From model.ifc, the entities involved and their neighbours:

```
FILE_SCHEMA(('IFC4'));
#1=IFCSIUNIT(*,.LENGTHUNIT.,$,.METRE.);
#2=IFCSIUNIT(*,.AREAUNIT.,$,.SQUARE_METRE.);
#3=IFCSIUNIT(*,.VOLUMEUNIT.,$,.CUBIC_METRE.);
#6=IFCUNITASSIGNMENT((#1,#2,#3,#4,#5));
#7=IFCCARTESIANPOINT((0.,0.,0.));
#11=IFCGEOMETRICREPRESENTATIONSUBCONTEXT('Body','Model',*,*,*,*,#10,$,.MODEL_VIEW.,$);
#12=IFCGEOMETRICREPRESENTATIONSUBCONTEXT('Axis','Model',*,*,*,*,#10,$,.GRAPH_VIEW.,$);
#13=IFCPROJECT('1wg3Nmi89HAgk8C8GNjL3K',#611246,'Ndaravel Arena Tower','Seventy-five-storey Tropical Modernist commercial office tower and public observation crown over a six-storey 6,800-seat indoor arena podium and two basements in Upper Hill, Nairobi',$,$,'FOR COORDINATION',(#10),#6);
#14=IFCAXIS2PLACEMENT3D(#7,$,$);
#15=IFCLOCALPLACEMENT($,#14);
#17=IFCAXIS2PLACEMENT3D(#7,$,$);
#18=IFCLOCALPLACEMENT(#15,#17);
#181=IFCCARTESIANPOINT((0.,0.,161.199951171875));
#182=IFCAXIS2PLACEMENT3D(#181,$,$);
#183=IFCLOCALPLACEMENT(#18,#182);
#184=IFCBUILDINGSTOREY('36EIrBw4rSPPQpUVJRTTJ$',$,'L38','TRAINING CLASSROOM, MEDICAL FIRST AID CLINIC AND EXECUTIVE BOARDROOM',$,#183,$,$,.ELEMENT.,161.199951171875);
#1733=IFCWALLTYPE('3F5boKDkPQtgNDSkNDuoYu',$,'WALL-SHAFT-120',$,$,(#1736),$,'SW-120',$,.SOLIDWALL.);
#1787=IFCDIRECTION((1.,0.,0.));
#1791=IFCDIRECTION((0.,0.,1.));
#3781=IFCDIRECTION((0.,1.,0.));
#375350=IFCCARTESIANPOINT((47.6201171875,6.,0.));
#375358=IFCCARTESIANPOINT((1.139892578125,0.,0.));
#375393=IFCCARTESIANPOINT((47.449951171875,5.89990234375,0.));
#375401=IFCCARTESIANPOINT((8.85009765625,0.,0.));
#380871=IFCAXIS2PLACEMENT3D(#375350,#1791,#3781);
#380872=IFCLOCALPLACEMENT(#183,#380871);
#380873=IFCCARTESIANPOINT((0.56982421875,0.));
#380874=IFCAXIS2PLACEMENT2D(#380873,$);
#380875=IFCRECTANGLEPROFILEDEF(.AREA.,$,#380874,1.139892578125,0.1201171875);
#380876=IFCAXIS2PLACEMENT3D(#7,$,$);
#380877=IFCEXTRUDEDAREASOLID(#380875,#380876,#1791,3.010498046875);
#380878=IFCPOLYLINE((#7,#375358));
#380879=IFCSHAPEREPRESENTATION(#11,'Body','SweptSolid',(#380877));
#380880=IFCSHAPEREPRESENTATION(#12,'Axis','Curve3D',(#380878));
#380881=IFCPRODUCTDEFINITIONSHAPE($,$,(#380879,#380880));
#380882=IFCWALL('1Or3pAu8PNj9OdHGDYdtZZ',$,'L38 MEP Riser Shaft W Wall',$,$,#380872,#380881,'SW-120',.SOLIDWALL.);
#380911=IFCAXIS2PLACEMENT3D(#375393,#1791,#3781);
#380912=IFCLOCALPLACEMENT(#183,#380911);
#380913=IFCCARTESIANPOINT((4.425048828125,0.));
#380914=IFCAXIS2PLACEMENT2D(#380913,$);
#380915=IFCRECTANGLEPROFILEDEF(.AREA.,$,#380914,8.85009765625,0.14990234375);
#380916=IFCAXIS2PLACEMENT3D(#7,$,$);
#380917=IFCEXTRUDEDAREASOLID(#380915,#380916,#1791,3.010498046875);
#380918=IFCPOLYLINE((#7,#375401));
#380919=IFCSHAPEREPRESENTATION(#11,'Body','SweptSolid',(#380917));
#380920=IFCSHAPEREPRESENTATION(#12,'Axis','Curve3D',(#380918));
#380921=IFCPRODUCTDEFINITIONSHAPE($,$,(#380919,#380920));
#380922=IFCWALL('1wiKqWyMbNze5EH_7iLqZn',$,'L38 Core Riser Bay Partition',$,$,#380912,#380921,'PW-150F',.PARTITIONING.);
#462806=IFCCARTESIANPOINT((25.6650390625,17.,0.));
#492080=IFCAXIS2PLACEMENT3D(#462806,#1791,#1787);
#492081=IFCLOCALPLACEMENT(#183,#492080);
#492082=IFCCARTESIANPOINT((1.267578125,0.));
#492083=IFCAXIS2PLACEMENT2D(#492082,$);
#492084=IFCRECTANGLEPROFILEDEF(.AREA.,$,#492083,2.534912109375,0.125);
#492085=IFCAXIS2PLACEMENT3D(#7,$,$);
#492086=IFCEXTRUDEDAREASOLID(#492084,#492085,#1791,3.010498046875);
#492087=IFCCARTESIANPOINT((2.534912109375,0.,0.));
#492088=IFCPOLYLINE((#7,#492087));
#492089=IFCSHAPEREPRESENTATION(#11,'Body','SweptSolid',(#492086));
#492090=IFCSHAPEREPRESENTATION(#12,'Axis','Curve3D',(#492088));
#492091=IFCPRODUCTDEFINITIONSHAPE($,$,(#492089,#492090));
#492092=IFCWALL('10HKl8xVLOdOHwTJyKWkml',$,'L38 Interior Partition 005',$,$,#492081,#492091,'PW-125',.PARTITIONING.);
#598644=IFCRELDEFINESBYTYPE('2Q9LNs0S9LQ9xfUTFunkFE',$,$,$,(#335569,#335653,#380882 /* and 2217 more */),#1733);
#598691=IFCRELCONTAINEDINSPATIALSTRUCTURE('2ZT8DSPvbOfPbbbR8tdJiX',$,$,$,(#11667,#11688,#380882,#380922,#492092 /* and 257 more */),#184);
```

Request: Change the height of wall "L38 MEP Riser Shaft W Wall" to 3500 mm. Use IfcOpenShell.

```python
import ifcopenshell
import ifcopenshell.geom
import ifcopenshell.util.representation
import ifcopenshell.util.shape

model = ifcopenshell.open("model.ifc")
settings = ifcopenshell.geom.settings()


def volume(element):
    """Net volume in cubic metres, openings subtracted."""
    shape = ifcopenshell.geom.create_shape(settings, element)
    return ifcopenshell.util.shape.get_volume(shape.geometry)


wall = model.by_guid("1Or3pAu8PNj9OdHGDYdtZZ")
before = volume(wall)

body = ifcopenshell.util.representation.get_representation(wall, "Model", "Body")
solid = body.Items[0]
old_height = solid.Depth
solid.Depth = 3.5
after = volume(wall)

print(f"height {old_height:g} -> {solid.Depth:g}, volume {before:.3f} -> {after:.3f} m3")

model.write("model_edited.ifc")
```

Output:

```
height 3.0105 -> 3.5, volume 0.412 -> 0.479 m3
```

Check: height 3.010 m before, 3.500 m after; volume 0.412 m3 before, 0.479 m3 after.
